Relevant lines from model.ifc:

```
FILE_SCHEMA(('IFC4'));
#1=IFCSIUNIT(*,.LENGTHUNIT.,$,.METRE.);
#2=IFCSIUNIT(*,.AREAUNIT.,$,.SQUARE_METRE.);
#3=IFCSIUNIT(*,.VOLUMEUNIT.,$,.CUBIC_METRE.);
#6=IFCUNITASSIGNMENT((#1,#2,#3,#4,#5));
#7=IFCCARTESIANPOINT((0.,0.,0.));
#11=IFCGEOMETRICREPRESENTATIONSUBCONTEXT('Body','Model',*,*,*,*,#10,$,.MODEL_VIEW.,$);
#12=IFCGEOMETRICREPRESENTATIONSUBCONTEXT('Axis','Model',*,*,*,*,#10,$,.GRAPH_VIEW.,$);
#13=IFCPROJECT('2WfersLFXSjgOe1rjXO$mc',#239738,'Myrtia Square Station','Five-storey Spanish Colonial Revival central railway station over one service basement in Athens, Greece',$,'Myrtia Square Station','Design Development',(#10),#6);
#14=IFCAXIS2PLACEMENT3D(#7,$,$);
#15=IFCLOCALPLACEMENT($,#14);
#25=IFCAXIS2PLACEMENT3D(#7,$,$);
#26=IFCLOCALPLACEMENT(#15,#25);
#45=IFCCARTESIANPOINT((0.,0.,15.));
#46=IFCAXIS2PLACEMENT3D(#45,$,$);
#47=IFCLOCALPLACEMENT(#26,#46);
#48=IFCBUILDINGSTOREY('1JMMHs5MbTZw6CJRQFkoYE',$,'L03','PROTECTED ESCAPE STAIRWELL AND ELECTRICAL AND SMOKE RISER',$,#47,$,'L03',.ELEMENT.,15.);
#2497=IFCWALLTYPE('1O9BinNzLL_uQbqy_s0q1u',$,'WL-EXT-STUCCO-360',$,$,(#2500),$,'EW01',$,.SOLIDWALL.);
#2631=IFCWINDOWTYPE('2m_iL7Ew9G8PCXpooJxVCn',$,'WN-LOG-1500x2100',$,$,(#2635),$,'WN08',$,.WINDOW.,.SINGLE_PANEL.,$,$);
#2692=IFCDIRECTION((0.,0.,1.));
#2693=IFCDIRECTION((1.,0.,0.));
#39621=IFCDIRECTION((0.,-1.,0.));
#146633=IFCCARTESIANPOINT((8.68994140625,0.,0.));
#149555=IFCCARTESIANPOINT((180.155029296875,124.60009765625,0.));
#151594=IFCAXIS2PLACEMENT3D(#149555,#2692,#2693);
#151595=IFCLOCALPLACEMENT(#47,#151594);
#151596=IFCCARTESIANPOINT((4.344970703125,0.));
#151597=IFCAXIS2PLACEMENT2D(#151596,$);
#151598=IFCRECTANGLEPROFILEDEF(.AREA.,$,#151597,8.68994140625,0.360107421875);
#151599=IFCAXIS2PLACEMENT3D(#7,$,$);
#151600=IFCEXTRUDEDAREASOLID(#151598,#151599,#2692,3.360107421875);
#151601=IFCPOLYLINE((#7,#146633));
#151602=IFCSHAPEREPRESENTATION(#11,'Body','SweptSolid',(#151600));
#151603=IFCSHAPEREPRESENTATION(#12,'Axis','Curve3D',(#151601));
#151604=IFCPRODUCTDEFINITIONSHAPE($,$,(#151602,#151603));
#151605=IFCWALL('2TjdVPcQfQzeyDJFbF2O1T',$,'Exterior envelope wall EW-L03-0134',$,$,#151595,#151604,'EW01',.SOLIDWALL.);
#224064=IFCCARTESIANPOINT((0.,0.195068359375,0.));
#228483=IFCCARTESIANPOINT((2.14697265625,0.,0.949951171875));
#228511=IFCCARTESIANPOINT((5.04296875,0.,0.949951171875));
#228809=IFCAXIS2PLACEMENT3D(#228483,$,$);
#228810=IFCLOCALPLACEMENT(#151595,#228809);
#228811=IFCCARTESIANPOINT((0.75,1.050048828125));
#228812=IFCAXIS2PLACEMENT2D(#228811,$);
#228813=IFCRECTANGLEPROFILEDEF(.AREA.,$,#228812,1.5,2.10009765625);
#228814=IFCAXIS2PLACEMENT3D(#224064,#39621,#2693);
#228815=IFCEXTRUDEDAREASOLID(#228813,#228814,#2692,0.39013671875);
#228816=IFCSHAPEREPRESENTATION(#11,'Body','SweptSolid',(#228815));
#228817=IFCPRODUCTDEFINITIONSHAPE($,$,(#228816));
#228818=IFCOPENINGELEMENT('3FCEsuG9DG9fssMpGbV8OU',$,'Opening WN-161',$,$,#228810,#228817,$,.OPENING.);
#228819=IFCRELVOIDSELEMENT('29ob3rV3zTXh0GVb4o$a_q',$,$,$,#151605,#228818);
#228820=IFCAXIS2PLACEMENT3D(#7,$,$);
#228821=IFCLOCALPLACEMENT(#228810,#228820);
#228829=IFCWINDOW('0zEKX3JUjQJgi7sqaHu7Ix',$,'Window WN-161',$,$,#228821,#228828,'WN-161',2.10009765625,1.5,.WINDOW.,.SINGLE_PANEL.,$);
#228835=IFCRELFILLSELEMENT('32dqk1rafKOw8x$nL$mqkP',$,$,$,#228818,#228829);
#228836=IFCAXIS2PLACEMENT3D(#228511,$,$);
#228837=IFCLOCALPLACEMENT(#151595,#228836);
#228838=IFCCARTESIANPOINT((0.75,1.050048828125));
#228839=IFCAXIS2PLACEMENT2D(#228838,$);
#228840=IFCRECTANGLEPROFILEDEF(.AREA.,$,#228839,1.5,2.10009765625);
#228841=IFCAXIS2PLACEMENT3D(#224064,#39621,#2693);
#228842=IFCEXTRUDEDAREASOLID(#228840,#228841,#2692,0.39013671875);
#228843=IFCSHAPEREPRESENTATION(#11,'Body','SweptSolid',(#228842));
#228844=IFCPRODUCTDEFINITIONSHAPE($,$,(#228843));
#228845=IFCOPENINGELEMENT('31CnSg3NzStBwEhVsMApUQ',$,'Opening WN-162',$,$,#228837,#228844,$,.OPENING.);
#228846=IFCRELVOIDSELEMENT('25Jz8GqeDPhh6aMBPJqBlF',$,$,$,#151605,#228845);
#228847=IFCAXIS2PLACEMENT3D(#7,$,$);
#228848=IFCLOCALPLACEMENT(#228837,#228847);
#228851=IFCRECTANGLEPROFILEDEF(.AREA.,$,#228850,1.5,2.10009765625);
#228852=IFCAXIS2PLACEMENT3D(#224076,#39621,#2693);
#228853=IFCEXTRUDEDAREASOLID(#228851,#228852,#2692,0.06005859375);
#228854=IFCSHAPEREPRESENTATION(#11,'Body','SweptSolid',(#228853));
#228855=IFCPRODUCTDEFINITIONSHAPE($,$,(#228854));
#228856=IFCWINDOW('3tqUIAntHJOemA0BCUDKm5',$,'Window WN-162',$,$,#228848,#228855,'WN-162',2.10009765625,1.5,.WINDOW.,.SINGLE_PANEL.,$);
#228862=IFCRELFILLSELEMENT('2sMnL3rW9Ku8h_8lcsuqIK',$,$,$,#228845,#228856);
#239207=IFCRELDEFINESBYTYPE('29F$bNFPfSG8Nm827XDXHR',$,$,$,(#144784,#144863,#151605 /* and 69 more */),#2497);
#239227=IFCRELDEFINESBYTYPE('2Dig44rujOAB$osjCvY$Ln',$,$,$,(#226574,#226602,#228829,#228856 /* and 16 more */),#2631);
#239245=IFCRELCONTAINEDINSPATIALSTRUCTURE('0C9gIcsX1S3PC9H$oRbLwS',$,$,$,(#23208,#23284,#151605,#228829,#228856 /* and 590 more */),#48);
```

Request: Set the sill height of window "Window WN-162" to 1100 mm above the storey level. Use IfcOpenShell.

```python
import numpy as np
import ifcopenshell
import ifcopenshell.api.geometry
import ifcopenshell.geom
import ifcopenshell.util.element
import ifcopenshell.util.placement
import ifcopenshell.util.shape
import ifcopenshell.util.unit

model = ifcopenshell.open("model.ifc")
unit_scale = ifcopenshell.util.unit.calculate_unit_scale(model)

window = model.by_guid("3tqUIAntHJOemA0BCUDKm5")
opening = window.FillsVoids[0].RelatingOpeningElement
storey = ifcopenshell.util.element.get_container(window, ifc_class="IfcBuildingStorey")
level = ifcopenshell.util.placement.get_local_placement(storey.ObjectPlacement)[2, 3]

# The opening's origin need not be at the sill, so measure its lowest point.
shape = ifcopenshell.geom.create_shape(ifcopenshell.geom.settings(), opening)
bottom = ifcopenshell.util.shape.get_shape_bottom_elevation(shape, shape.geometry) / unit_scale
dz = level + 1.1 / unit_scale - bottom

shift = np.array([0.0, 0.0, dz])
# The window is placed relative to its opening, so it follows when the opening moves.
matrix = ifcopenshell.util.placement.get_local_placement(opening.ObjectPlacement)
matrix[:3, 3] += shift
ifcopenshell.api.geometry.edit_object_placement(
    model, product=opening, matrix=matrix, is_si=False, should_transform_children=True
)

print(f"moved by {dz * unit_scale:+.3f} m")

model.write("model_updated.ifc")
```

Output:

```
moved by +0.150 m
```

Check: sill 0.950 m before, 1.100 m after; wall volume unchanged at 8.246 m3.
